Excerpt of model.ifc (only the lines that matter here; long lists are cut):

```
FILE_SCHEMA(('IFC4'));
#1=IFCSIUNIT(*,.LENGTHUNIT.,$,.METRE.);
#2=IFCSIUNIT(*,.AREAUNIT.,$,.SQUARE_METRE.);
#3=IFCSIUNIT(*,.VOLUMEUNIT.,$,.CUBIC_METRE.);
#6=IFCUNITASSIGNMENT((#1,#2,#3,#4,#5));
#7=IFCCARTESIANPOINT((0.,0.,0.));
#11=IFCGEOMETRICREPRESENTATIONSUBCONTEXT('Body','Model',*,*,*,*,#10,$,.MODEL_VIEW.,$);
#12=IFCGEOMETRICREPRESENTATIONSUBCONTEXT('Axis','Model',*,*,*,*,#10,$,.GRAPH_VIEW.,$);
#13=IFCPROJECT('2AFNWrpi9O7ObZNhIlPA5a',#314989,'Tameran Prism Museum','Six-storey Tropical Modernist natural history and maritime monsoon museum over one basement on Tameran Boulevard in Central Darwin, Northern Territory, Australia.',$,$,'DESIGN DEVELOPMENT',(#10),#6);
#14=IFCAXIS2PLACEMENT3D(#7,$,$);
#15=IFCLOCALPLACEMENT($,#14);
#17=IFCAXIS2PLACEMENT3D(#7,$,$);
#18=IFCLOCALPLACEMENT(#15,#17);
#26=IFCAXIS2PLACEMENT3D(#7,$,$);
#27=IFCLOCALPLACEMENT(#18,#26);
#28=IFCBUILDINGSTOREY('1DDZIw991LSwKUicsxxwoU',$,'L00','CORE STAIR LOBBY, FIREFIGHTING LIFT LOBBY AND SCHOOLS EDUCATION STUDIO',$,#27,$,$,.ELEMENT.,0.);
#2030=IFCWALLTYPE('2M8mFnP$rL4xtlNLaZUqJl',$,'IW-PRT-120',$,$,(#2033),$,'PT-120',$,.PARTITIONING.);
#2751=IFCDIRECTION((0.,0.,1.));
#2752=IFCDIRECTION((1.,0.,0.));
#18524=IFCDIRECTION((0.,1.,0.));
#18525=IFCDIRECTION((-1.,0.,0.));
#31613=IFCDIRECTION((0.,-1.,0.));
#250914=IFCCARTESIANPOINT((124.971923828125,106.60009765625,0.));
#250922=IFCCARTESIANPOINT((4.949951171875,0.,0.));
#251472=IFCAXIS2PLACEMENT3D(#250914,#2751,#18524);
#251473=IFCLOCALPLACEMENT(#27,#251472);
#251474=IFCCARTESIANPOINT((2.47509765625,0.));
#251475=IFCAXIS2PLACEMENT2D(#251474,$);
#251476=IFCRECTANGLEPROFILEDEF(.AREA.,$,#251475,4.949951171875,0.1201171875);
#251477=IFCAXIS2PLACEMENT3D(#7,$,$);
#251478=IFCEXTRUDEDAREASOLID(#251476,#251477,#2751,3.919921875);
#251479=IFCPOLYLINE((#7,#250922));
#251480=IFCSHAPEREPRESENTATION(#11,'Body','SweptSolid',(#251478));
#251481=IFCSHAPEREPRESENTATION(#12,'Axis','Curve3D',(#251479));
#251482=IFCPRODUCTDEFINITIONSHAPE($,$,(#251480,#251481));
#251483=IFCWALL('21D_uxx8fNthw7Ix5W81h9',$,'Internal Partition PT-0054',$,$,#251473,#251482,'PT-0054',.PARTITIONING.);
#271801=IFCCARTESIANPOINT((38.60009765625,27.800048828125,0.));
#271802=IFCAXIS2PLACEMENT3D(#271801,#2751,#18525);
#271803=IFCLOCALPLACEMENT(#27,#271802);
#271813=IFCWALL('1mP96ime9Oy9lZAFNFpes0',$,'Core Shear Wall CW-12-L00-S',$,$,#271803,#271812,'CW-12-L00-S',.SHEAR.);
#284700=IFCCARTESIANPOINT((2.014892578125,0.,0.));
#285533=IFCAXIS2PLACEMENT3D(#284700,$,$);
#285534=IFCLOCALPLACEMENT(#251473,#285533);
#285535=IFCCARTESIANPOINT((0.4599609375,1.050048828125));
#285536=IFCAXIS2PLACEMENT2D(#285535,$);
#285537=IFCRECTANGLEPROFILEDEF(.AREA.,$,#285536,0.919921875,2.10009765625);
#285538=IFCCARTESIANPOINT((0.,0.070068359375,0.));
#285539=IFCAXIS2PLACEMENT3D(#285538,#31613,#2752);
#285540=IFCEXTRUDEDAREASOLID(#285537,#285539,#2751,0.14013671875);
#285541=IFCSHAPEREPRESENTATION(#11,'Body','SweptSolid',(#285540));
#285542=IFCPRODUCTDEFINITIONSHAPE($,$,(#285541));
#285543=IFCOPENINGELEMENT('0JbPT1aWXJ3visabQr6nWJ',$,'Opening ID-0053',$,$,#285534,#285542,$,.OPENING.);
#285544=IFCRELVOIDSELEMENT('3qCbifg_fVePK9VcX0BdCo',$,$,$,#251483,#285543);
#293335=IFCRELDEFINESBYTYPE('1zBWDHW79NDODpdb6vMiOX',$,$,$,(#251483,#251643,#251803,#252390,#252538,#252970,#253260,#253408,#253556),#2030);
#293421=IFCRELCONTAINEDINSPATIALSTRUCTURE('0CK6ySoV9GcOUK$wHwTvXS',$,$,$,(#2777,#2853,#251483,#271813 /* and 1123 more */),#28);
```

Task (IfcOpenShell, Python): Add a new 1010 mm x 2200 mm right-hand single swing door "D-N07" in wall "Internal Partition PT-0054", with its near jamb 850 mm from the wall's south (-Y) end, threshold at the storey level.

```python
import numpy as np
import ifcopenshell
import ifcopenshell.api.feature
import ifcopenshell.api.geometry
import ifcopenshell.api.root
import ifcopenshell.api.spatial
import ifcopenshell.geom
import ifcopenshell.util.element
import ifcopenshell.util.placement
import ifcopenshell.util.representation
import ifcopenshell.util.shape
import ifcopenshell.util.unit

model = ifcopenshell.open("model.ifc")
unit_scale = ifcopenshell.util.unit.calculate_unit_scale(model)
settings = ifcopenshell.geom.settings()


def volume(element):
    """Net volume in cubic metres, openings subtracted."""
    shape = ifcopenshell.geom.create_shape(settings, element)
    return ifcopenshell.util.shape.get_volume(shape.geometry)


wall = model.by_guid("21D_uxx8fNthw7Ix5W81h9")
storey = ifcopenshell.util.element.get_container(wall, ifc_class="IfcBuildingStorey")
context = ifcopenshell.util.representation.get_context(model, "Model", "Body", "MODEL_VIEW")
before = volume(wall)

width, height, from_end, sill = 1.01, 2.2, 0.85, 0.0  # metres

# The wall runs along its own X axis, and the end named is its -X end.
wall_shape = ifcopenshell.geom.create_shape(settings, wall)
x, y, z = ifcopenshell.util.shape.get_vertices(wall_shape.geometry).T
start = x.min() + from_end
face, thickness = float(y.min()), float(y.max() - y.min())
wall_matrix = ifcopenshell.util.placement.get_local_placement(wall.ObjectPlacement)
level = ifcopenshell.util.placement.get_local_placement(storey.ObjectPlacement)[2, 3]


def in_wall(x, y):
    """Placement at x, y metres in the wall's axes, at sill height."""
    matrix = wall_matrix.copy()
    matrix[:, 3] = wall_matrix @ np.array([x / unit_scale, y / unit_scale, 0.0, 1.0])
    matrix[2, 3] = level + sill / unit_scale
    return matrix


# Opening: a box that overshoots both wall faces by 50 mm.
opening = ifcopenshell.api.root.create_entity(model, ifc_class="IfcOpeningElement", predefined_type="OPENING")
box = ifcopenshell.api.geometry.add_wall_representation(
    model, context=context, length=width, height=height, thickness=thickness + 0.1
)
ifcopenshell.api.geometry.assign_representation(model, product=opening, representation=box)
ifcopenshell.api.geometry.edit_object_placement(model, product=opening, matrix=in_wall(start, face - 0.05), is_si=False)
ifcopenshell.api.feature.add_feature(model, feature=opening, element=wall)

door = ifcopenshell.api.root.create_entity(model, ifc_class="IfcDoor", name="D-N07", predefined_type="DOOR")
door.OverallWidth, door.OverallHeight = width / unit_scale, height / unit_scale
door.OperationType = "SINGLE_SWING_RIGHT"
body = ifcopenshell.api.geometry.add_door_representation(
    model,
    context=context,
    overall_width=door.OverallWidth,
    overall_height=door.OverallHeight,
    operation_type="SINGLE_SWING_RIGHT",
    lining_properties={"LiningDepth": thickness / unit_scale, "ThresholdDepth": thickness / unit_scale},
)
ifcopenshell.api.geometry.assign_representation(model, product=door, representation=body)
ifcopenshell.api.spatial.assign_container(model, products=[door], relating_structure=storey)
ifcopenshell.api.feature.add_filling(model, opening=opening, element=door)

# The lining spans the wall, so the door starts at the wall face.
ifcopenshell.api.geometry.edit_object_placement(model, product=door, matrix=in_wall(start, face), is_si=False)

after = volume(wall)

print(f"wall volume {before:.3f} -> {after:.3f} m3")

model.write("model-out.ifc")
```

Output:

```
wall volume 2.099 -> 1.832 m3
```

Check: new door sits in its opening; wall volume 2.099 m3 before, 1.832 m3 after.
